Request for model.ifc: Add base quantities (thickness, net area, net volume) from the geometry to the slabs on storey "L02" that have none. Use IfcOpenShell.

First a look at what the model holds.

```python
import ifcopenshell
import ifcopenshell.util.element
import ifcopenshell.util.unit

model = ifcopenshell.open("model.ifc")
print(model.schema)
for unit_type in ("LENGTHUNIT", "AREAUNIT", "VOLUMEUNIT"):
    print(unit_type, ifcopenshell.util.unit.calculate_unit_scale(model, unit_type))
storey = next(s for s in model.by_type("IfcBuildingStorey") if s.Name == "L02")
slabs = [e for e in ifcopenshell.util.element.get_decomposition(storey) if e.is_a("IfcSlab")]
for e in sorted(slabs, key=lambda e: e.id()):
    print(e.id(), e.is_a(), e.Name, list(ifcopenshell.util.element.get_psets(e, qtos_only=True)), sep=" | ")
```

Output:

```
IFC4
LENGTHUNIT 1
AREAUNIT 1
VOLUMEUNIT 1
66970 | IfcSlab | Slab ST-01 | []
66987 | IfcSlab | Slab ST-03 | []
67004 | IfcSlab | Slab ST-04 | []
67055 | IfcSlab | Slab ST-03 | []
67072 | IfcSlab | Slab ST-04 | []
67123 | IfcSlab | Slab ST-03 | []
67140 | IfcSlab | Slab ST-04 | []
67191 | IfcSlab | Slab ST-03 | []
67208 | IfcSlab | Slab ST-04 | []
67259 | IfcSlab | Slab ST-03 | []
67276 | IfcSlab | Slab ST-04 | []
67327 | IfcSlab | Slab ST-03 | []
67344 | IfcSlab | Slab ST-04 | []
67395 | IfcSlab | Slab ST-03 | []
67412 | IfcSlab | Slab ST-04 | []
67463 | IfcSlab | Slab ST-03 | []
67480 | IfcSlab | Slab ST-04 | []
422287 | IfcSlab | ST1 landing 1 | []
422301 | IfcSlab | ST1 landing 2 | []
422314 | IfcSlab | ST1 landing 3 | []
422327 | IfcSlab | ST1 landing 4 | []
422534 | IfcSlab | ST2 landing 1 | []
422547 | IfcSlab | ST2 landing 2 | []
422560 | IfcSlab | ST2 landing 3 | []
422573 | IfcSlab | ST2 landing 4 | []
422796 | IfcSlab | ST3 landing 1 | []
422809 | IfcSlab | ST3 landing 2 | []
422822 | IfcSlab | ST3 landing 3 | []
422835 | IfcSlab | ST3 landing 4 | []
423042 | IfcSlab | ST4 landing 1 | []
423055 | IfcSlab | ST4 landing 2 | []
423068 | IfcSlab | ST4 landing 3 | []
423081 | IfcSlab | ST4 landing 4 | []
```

```python
import ifcopenshell
import ifcopenshell.api.pset
import ifcopenshell.geom
import ifcopenshell.util.element
import ifcopenshell.util.shape
import ifcopenshell.util.unit

model = ifcopenshell.open("model.ifc")
unit_scale = ifcopenshell.util.unit.calculate_unit_scale(model)
area_scale = ifcopenshell.util.unit.calculate_unit_scale(model, "AREAUNIT")
volume_scale = ifcopenshell.util.unit.calculate_unit_scale(model, "VOLUMEUNIT")
settings = ifcopenshell.geom.settings()

storey = next(s for s in model.by_type("IfcBuildingStorey") if s.Name == "L02")
slabs = [e for e in ifcopenshell.util.element.get_decomposition(storey) if e.is_a("IfcSlab")]

for e in sorted(slabs, key=lambda e: e.id()):
    if ifcopenshell.util.element.get_psets(e, qtos_only=True, should_inherit=False):
        continue
    # Geometry comes back in metres, in the element's own axes.
    shape = ifcopenshell.geom.create_shape(settings, e)
    values = {
        "Width": ifcopenshell.util.shape.get_z(shape.geometry) / unit_scale,
        "NetArea": ifcopenshell.util.shape.get_footprint_area(shape.geometry) / area_scale,
        "NetVolume": ifcopenshell.util.shape.get_volume(shape.geometry) / volume_scale,
    }
    qto = ifcopenshell.api.pset.add_qto(model, product=e, name="Qto_SlabBaseQuantities")
    ifcopenshell.api.pset.edit_qto(model, qto=qto, properties=values)
    print(e.id(), {k: round(v, 3) for k, v in values.items()})

model.write("model_v2.ifc")
```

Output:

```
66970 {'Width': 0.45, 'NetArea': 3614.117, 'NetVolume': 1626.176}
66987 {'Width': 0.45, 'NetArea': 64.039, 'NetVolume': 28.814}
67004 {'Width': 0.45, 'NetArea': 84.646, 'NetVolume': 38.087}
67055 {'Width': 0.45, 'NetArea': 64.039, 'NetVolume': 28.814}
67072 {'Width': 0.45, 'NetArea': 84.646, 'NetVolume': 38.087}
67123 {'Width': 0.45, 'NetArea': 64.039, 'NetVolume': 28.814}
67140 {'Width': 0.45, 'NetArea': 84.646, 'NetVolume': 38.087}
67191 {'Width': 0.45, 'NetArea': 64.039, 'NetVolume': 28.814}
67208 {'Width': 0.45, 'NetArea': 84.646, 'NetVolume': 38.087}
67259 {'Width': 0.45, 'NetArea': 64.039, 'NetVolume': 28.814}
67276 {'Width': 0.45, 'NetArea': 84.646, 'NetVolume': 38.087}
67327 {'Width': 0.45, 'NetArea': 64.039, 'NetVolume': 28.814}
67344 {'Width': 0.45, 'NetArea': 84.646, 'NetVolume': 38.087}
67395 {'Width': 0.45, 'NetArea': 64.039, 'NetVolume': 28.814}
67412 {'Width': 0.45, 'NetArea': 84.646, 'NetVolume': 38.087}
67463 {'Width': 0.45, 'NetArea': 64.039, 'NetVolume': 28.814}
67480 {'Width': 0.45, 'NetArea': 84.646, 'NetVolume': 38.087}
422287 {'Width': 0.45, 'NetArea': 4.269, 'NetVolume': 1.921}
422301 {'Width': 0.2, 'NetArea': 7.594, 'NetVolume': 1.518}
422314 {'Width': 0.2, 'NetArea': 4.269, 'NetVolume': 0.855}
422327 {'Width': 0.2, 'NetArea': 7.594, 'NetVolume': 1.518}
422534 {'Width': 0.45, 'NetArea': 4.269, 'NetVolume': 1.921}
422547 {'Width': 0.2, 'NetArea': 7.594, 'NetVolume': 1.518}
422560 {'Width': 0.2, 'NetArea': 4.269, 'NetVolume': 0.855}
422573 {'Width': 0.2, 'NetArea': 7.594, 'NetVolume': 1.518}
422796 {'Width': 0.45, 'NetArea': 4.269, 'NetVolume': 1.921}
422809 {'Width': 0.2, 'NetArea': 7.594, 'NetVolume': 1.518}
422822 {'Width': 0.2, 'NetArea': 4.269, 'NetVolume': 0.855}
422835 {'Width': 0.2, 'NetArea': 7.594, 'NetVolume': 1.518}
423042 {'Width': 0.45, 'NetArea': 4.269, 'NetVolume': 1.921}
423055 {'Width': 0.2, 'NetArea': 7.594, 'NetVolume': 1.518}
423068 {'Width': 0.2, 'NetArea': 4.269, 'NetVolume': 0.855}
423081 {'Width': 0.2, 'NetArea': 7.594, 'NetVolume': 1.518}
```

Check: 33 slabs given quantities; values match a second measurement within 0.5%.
